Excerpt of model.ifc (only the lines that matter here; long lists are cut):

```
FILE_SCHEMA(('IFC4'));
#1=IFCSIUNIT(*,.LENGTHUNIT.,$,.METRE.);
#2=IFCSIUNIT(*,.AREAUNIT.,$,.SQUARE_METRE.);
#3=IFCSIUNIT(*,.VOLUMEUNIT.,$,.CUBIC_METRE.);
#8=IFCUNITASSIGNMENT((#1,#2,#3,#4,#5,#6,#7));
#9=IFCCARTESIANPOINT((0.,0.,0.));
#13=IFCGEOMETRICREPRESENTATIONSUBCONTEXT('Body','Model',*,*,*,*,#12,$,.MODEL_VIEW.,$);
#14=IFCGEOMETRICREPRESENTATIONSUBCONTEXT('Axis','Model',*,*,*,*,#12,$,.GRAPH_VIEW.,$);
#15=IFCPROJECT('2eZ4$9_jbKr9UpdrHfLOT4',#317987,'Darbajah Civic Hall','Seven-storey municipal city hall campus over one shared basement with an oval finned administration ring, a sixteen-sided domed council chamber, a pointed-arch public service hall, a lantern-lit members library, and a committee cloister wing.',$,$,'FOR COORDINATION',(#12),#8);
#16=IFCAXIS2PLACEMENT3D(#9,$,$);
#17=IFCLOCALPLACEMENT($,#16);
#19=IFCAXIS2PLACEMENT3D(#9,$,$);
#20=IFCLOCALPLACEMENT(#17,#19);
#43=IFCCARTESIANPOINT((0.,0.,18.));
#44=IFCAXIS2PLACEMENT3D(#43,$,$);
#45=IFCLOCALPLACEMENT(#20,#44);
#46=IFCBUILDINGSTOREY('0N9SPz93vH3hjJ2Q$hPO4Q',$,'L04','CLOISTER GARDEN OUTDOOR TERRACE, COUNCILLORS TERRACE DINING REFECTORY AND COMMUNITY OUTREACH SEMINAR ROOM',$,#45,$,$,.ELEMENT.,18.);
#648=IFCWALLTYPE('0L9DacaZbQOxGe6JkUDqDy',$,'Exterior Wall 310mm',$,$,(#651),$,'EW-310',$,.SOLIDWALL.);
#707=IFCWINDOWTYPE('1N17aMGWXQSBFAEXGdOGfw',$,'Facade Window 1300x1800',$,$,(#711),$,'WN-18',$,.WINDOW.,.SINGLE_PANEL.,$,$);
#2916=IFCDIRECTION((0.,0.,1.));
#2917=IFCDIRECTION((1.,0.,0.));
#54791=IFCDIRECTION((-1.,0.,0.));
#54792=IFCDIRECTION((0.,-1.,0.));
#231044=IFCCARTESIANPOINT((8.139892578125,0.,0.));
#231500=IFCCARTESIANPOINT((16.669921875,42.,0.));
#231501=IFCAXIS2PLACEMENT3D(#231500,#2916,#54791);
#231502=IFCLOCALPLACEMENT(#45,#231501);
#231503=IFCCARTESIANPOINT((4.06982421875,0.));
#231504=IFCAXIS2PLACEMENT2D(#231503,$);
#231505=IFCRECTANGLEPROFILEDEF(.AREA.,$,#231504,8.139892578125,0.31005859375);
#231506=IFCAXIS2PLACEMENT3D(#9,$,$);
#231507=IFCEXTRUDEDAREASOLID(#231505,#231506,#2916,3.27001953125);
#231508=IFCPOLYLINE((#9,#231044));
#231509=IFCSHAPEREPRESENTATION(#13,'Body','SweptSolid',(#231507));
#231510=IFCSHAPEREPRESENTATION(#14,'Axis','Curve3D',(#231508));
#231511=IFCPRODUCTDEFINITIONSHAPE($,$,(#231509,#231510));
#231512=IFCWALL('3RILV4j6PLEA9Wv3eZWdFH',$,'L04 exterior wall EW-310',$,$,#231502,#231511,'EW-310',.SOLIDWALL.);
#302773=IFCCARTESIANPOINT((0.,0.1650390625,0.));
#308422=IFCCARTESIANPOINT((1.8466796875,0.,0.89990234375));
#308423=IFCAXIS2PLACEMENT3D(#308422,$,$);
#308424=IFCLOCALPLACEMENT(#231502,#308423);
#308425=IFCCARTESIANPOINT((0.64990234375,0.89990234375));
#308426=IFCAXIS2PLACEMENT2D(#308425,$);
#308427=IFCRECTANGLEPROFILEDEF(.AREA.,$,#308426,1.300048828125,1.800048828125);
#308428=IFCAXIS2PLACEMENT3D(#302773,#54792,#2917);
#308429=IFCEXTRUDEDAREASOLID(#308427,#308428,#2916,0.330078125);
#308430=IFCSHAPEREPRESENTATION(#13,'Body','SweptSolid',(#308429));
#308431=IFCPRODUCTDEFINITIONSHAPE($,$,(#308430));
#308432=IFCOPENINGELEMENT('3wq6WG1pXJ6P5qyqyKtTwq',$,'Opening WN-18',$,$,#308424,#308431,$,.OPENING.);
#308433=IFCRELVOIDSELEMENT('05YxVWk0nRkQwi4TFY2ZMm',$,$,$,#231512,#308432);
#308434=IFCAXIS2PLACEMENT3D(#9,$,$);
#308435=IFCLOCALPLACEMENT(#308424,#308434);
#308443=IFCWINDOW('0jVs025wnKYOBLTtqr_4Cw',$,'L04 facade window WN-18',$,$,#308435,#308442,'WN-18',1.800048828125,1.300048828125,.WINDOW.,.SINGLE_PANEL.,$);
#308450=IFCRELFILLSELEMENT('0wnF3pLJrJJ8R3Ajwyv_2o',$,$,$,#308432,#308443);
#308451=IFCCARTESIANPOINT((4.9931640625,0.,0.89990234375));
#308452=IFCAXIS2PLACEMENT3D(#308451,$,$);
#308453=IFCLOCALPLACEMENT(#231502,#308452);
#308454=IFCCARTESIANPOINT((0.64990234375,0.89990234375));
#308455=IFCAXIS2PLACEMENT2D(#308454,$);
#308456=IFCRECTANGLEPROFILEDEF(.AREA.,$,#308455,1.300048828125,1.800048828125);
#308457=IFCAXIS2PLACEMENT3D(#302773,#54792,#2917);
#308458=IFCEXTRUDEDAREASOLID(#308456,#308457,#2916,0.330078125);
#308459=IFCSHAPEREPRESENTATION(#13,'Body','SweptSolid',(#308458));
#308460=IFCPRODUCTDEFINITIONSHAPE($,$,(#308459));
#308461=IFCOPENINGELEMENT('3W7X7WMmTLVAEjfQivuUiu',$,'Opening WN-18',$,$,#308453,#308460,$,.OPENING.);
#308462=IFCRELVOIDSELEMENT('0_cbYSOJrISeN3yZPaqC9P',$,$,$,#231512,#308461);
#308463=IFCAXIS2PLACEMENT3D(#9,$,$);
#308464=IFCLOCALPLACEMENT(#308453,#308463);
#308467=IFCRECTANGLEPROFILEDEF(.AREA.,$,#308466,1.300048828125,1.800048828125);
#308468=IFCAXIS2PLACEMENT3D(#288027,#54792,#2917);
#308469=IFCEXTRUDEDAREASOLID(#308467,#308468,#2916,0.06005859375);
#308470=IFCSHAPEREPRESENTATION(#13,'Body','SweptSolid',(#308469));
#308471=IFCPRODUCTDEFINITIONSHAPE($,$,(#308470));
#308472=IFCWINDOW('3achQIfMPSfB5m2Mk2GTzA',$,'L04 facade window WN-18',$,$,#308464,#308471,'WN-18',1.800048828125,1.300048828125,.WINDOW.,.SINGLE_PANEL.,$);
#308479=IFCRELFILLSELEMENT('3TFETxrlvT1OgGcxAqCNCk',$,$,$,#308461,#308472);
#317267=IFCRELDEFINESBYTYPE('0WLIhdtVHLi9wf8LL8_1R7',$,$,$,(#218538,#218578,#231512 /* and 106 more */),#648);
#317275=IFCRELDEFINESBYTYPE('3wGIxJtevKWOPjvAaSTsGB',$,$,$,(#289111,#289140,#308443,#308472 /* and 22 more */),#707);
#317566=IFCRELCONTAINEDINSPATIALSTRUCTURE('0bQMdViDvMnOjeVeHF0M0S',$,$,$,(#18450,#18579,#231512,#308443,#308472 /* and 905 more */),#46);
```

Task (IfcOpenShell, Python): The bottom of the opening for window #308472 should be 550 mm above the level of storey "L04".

```python
import numpy as np
import ifcopenshell
import ifcopenshell.api.geometry
import ifcopenshell.geom
import ifcopenshell.util.element
import ifcopenshell.util.placement
import ifcopenshell.util.shape
import ifcopenshell.util.unit

model = ifcopenshell.open("model.ifc")
unit_scale = ifcopenshell.util.unit.calculate_unit_scale(model)

window = model.by_guid("3achQIfMPSfB5m2Mk2GTzA")
opening = window.FillsVoids[0].RelatingOpeningElement
storey = ifcopenshell.util.element.get_container(window, ifc_class="IfcBuildingStorey")
level = ifcopenshell.util.placement.get_local_placement(storey.ObjectPlacement)[2, 3]

# The opening's origin need not be at the sill, so measure its lowest point.
shape = ifcopenshell.geom.create_shape(ifcopenshell.geom.settings(), opening)
bottom = ifcopenshell.util.shape.get_shape_bottom_elevation(shape, shape.geometry) / unit_scale
dz = level + 0.55 - bottom

shift = np.array([0.0, 0.0, dz])
# The window is placed relative to its opening, so it follows when the opening moves.
matrix = ifcopenshell.util.placement.get_local_placement(opening.ObjectPlacement)
matrix[:3, 3] += shift
ifcopenshell.api.geometry.edit_object_placement(
    model, product=opening, matrix=matrix, is_si=False, should_transform_children=True
)

print(f"moved by {dz * unit_scale:+.3f} m")

model.write("model_rev.ifc")
```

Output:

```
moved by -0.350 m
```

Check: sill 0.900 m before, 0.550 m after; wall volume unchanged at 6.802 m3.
